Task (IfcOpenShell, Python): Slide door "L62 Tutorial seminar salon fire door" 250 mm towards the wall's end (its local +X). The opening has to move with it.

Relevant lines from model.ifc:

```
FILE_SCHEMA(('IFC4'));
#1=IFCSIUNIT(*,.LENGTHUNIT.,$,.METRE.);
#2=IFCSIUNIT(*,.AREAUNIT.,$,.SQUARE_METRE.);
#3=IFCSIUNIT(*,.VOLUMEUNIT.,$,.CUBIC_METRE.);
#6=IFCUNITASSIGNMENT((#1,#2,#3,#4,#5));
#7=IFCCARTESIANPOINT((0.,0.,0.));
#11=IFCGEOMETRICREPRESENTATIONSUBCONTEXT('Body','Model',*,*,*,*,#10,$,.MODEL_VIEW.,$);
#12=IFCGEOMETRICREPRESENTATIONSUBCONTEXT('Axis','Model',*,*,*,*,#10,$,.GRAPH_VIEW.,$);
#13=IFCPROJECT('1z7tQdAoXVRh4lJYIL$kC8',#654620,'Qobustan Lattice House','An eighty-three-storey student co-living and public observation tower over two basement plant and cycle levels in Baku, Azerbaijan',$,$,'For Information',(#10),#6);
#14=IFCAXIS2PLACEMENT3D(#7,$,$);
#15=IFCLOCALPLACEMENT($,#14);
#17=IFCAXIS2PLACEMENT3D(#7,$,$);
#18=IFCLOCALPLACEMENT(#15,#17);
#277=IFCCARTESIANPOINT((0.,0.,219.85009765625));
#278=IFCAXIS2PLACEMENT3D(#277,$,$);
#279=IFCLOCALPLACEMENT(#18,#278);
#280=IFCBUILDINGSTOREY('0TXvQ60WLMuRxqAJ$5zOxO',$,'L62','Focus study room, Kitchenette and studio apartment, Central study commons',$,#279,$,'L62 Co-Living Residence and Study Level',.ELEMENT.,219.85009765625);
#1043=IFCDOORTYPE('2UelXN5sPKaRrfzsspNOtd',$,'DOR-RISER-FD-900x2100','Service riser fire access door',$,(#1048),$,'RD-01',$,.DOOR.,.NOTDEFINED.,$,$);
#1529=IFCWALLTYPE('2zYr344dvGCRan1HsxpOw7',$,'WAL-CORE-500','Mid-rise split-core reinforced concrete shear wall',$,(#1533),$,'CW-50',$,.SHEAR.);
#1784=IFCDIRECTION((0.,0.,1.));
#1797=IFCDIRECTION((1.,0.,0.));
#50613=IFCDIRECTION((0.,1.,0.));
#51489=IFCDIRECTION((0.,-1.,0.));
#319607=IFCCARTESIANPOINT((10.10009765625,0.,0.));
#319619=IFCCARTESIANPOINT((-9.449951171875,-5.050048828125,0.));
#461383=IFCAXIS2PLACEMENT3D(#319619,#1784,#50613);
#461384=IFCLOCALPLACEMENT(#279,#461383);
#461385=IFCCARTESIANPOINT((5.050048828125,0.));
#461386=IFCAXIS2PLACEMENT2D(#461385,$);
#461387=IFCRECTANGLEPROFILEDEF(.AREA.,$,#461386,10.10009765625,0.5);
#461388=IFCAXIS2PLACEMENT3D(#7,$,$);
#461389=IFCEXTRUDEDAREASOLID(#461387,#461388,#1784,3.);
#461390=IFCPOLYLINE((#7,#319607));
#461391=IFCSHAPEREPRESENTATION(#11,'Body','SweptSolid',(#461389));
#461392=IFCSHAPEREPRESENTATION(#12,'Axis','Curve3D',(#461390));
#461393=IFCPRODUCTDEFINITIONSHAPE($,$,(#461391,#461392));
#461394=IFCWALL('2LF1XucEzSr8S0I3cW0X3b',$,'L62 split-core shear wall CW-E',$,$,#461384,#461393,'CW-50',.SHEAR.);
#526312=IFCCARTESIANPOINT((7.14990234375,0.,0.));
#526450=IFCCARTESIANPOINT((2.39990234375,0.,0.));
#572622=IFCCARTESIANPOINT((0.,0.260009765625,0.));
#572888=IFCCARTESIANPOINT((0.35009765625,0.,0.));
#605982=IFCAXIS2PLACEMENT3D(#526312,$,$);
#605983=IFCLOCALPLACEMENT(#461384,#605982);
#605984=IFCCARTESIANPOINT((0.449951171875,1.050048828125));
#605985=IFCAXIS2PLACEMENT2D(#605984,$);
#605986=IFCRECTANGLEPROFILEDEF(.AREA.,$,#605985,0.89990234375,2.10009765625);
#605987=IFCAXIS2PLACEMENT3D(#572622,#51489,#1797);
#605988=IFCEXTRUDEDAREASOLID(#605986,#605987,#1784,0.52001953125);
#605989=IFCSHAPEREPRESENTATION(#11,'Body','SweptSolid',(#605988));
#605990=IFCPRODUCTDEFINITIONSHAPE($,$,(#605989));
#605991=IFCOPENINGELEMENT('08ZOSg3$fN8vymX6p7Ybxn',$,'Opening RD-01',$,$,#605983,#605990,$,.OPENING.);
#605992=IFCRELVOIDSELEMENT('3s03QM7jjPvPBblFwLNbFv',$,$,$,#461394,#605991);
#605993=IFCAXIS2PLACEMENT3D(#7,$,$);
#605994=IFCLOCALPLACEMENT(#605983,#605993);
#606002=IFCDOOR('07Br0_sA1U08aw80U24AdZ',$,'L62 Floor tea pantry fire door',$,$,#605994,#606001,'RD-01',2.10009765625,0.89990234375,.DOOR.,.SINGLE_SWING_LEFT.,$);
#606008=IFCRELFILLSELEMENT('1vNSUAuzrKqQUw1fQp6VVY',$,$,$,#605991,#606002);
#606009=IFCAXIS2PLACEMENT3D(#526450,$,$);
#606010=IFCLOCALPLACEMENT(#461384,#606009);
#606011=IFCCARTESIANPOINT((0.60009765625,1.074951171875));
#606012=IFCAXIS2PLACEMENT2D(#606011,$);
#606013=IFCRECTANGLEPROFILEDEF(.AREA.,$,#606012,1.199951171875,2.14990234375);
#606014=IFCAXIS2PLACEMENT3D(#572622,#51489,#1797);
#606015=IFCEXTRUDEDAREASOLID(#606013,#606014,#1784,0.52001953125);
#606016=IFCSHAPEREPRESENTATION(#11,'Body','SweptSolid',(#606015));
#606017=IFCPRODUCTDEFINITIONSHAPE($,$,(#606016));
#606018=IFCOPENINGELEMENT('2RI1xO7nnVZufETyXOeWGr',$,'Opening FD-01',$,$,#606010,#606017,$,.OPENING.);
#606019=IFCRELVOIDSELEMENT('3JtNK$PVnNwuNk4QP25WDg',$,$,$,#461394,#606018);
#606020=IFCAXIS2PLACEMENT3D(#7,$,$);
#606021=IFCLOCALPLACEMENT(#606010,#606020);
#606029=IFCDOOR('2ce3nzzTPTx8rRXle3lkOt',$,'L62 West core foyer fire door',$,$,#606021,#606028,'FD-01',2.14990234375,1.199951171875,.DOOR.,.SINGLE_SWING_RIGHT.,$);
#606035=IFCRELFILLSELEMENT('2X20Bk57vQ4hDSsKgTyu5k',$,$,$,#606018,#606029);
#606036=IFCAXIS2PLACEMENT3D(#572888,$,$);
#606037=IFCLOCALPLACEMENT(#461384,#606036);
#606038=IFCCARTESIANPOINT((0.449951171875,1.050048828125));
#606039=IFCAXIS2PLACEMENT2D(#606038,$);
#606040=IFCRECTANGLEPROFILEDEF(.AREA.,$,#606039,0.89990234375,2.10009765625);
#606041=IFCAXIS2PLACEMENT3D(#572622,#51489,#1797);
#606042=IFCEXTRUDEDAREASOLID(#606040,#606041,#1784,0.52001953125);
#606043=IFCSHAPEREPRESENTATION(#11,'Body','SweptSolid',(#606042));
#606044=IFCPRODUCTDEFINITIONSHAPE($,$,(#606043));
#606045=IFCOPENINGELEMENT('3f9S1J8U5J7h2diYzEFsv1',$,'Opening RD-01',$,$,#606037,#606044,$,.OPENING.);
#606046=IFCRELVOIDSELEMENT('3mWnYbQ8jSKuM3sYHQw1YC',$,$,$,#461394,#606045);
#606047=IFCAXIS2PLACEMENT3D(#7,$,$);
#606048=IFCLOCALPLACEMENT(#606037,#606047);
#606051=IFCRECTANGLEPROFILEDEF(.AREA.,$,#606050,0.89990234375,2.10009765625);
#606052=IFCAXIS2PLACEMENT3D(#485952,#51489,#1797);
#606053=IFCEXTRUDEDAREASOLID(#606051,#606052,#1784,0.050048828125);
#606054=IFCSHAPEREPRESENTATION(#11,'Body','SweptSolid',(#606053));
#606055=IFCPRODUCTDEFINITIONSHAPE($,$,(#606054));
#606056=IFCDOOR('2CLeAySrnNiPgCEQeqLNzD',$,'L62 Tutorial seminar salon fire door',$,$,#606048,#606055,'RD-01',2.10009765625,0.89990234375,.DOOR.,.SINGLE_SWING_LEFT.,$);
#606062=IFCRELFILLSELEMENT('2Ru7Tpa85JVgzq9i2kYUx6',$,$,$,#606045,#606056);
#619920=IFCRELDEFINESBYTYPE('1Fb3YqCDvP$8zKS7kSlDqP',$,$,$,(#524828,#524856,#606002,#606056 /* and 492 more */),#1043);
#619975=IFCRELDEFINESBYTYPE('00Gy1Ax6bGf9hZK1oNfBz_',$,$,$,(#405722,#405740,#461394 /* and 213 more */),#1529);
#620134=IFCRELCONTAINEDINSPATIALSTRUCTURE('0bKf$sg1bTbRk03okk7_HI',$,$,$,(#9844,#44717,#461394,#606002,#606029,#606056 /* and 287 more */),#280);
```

```python
import ifcopenshell
import ifcopenshell.api.geometry
import ifcopenshell.util.placement

model = ifcopenshell.open("model.ifc")

door = model.by_guid("2CLeAySrnNiPgCEQeqLNzD")
opening = door.FillsVoids[0].RelatingOpeningElement
wall = opening.VoidsElements[0].RelatingBuildingElement

wall_matrix = ifcopenshell.util.placement.get_local_placement(wall.ObjectPlacement)
shift = wall_matrix[:3, 0] * 0.25
before = ifcopenshell.util.placement.get_local_placement(door.ObjectPlacement)[:3, 3].copy()

# The door is placed relative to its opening, so it follows when the opening moves.
matrix = ifcopenshell.util.placement.get_local_placement(opening.ObjectPlacement)
matrix[:3, 3] += shift
ifcopenshell.api.geometry.edit_object_placement(
    model, product=opening, matrix=matrix, is_si=False, should_transform_children=True
)

after = ifcopenshell.util.placement.get_local_placement(door.ObjectPlacement)[:3, 3]
print("door moved by", (after - before).round(3) + 0.0)

model.write("model_updated.ifc")
```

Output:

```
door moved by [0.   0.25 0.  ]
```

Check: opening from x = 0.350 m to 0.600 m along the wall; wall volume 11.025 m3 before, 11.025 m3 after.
